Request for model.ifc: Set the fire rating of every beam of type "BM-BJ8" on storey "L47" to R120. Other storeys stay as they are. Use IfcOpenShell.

First a look at what the model holds.

```python
import ifcopenshell
import ifcopenshell.util.element

model = ifcopenshell.open("model.ifc")
print(model.schema)
storey = next(s for s in model.by_type("IfcBuildingStorey") if s.Name == "L47")
beams = [e for e in ifcopenshell.util.element.get_decomposition(storey) if e.is_a("IfcBeam")]
seen = {}
for e in beams:
    element_type = ifcopenshell.util.element.get_type(e)
    key = (element_type.Name if element_type != e and element_type else None, ifcopenshell.util.element.get_pset(e, "Pset_BeamCommon", "FireRating"))
    seen[key] = seen.get(key, 0) + 1
for (name, value), count in sorted(seen.items(), key=str):
    print(count, "x", name, "|", value)
```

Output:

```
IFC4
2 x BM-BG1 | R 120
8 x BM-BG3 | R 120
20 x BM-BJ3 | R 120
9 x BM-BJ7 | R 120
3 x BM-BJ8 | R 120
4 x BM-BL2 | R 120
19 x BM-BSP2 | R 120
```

```python
import ifcopenshell
import ifcopenshell.api.pset
import ifcopenshell.util.element

model = ifcopenshell.open("model.ifc")

storey = next(s for s in model.by_type("IfcBuildingStorey") if s.Name == "L47")
beams = [e for e in ifcopenshell.util.element.get_decomposition(storey) if e.is_a("IfcBeam")]

count = 0
for e in beams:
    element_type = ifcopenshell.util.element.get_type(e)
    if element_type in (None, e) or element_type.Name != "BM-BJ8":
        continue
    found = ifcopenshell.util.element.get_pset(e, "Pset_BeamCommon", should_inherit=False)
    if found:
        pset = model.by_id(found["id"])
        if len(ifcopenshell.util.element.get_elements_by_pset(pset)) > 1:
            pset = ifcopenshell.api.pset.unshare_pset(model, products=[e], pset=pset)[0]
    else:
        pset = ifcopenshell.api.pset.add_pset(model, product=e, name="Pset_BeamCommon")
    ifcopenshell.api.pset.edit_pset(model, pset=pset, properties={"FireRating": "R120"})
    count += 1

print(count, "beams updated")

model.write("model_v2.ifc")
```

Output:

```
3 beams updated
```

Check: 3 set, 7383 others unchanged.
